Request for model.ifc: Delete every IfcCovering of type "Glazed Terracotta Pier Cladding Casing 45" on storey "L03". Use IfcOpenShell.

First a look at what the model holds.

```python
import ifcopenshell
import ifcopenshell.util.element

model = ifcopenshell.open("model.ifc")
print(model.schema)
storey = next(s for s in model.by_type("IfcBuildingStorey") if s.Name == "L03")
coverings = [e for e in ifcopenshell.util.element.get_decomposition(storey) if e.is_a("IfcCovering")]
seen = {}
for e in coverings:
    element_type = ifcopenshell.util.element.get_type(e)
    name = element_type.Name if element_type not in (None, e) else None
    seen[name] = seen.get(name, 0) + 1
for name, count in sorted(seen.items(), key=str):
    print(count, "x", name)
```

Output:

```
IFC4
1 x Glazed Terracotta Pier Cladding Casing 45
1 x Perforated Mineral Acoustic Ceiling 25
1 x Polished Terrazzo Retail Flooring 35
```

```python
import ifcopenshell
import ifcopenshell.api.root
import ifcopenshell.util.element

model = ifcopenshell.open("model.ifc")

storey = next(s for s in model.by_type("IfcBuildingStorey") if s.Name == "L03")
coverings = [e for e in ifcopenshell.util.element.get_decomposition(storey) if e.is_a("IfcCovering")]
targets = [e for e in coverings if (t := ifcopenshell.util.element.get_type(e)) not in (None, e) and t.Name == "Glazed Terracotta Pier Cladding Casing 45"]

for e in targets:
    ifcopenshell.api.root.remove_product(model, product=e)
print(len(targets), "removed")

model.write("model_v2.ifc")
```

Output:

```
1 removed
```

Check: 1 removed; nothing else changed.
